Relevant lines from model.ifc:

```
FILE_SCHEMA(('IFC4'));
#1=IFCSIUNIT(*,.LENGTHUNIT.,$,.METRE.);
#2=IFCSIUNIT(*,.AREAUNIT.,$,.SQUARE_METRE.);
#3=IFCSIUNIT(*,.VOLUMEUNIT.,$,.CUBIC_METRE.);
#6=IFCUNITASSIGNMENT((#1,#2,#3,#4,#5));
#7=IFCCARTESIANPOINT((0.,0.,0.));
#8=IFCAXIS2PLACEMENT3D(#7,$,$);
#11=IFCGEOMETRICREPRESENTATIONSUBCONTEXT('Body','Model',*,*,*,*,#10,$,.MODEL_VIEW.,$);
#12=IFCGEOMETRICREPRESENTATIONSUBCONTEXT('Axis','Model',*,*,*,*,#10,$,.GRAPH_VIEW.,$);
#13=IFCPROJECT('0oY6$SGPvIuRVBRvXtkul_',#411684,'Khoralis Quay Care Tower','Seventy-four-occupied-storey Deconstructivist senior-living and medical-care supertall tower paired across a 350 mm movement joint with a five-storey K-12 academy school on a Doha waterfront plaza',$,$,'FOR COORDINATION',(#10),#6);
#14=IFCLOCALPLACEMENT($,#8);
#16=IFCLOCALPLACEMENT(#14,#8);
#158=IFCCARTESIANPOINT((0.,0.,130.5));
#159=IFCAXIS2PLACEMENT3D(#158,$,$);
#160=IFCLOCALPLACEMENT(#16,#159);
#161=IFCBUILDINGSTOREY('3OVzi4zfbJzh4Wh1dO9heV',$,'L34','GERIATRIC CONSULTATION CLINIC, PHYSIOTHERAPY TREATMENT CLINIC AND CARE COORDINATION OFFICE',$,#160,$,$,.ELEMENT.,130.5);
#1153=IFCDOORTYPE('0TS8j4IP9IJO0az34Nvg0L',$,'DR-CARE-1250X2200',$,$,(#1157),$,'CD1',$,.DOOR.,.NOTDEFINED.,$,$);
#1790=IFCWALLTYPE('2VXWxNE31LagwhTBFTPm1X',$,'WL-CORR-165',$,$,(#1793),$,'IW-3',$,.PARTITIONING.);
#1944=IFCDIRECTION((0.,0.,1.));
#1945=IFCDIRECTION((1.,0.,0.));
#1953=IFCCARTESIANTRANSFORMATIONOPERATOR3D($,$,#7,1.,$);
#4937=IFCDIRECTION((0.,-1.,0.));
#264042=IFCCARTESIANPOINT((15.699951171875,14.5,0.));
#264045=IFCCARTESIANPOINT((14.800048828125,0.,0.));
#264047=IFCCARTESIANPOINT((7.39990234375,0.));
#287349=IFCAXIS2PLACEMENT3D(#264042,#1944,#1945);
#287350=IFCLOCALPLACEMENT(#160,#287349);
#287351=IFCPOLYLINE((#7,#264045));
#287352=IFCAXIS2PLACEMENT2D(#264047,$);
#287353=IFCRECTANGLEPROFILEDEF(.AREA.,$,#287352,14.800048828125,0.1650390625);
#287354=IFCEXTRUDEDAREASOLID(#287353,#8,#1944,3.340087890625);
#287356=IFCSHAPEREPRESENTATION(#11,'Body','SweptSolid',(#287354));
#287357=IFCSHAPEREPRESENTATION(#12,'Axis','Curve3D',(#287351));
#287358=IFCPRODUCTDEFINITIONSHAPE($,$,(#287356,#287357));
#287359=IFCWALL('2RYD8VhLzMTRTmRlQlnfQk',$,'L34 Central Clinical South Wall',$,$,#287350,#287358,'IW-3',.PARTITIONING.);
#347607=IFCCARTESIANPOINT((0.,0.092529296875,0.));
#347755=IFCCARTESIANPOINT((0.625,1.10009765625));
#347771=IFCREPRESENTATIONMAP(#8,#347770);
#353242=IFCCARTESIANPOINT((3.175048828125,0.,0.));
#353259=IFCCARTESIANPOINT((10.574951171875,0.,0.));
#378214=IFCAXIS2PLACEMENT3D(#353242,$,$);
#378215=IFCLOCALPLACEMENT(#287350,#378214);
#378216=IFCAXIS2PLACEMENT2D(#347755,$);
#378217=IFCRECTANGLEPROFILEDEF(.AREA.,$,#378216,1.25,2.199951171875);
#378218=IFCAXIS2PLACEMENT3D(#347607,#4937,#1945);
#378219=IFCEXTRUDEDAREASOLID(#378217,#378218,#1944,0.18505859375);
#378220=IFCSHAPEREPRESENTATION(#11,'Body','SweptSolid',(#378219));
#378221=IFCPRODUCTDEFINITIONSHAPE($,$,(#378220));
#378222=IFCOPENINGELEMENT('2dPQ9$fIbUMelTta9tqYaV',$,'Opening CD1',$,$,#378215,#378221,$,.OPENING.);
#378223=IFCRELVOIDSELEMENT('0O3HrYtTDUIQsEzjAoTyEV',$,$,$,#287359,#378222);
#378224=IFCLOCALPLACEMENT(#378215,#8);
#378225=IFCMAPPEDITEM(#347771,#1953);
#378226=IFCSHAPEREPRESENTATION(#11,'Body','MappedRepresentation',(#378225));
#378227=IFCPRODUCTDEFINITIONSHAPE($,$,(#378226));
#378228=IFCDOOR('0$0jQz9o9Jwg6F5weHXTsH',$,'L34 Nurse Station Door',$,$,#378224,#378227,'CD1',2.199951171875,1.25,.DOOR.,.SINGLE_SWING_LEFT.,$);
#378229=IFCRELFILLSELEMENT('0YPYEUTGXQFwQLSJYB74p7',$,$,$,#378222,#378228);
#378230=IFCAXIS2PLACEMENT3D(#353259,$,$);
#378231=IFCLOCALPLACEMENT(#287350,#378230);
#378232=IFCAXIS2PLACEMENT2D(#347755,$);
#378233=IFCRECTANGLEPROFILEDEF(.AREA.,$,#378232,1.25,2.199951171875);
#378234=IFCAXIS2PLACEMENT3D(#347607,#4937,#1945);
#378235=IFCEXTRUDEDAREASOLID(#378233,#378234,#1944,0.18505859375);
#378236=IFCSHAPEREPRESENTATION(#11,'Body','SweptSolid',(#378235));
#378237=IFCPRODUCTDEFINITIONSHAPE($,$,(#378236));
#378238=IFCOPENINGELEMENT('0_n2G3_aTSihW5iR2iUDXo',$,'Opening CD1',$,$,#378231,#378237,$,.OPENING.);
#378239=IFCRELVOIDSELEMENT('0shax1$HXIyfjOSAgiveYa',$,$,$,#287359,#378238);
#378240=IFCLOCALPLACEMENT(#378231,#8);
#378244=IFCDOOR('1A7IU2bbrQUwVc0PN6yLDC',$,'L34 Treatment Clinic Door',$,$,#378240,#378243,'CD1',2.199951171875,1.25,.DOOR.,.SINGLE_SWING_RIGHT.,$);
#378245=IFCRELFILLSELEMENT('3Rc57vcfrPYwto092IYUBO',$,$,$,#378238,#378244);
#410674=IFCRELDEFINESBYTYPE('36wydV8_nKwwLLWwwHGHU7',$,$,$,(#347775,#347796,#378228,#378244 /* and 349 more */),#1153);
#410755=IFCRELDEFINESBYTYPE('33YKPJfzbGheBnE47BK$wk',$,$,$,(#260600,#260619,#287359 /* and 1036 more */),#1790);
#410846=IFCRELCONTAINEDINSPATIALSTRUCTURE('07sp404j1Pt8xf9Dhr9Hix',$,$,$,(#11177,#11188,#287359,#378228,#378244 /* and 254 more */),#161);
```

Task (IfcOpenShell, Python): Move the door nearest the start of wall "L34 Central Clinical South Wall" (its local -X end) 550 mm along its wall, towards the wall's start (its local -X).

```python
import ifcopenshell
import ifcopenshell.api.geometry
import ifcopenshell.util.placement

model = ifcopenshell.open("model.ifc")

door = model.by_guid("0$0jQz9o9Jwg6F5weHXTsH")
opening = door.FillsVoids[0].RelatingOpeningElement
wall = opening.VoidsElements[0].RelatingBuildingElement

wall_matrix = ifcopenshell.util.placement.get_local_placement(wall.ObjectPlacement)
shift = wall_matrix[:3, 0] * -0.55
before = ifcopenshell.util.placement.get_local_placement(door.ObjectPlacement)[:3, 3].copy()

# The door is placed relative to its opening, so it follows when the opening moves.
matrix = ifcopenshell.util.placement.get_local_placement(opening.ObjectPlacement)
matrix[:3, 3] += shift
ifcopenshell.api.geometry.edit_object_placement(
    model, product=opening, matrix=matrix, is_si=False, should_transform_children=True
)

after = ifcopenshell.util.placement.get_local_placement(door.ObjectPlacement)[:3, 3]
print("door moved by", (after - before).round(3) + 0.0)

model.write("model_rev.ifc")
```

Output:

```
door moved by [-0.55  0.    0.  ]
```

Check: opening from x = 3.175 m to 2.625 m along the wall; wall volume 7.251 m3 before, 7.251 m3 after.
